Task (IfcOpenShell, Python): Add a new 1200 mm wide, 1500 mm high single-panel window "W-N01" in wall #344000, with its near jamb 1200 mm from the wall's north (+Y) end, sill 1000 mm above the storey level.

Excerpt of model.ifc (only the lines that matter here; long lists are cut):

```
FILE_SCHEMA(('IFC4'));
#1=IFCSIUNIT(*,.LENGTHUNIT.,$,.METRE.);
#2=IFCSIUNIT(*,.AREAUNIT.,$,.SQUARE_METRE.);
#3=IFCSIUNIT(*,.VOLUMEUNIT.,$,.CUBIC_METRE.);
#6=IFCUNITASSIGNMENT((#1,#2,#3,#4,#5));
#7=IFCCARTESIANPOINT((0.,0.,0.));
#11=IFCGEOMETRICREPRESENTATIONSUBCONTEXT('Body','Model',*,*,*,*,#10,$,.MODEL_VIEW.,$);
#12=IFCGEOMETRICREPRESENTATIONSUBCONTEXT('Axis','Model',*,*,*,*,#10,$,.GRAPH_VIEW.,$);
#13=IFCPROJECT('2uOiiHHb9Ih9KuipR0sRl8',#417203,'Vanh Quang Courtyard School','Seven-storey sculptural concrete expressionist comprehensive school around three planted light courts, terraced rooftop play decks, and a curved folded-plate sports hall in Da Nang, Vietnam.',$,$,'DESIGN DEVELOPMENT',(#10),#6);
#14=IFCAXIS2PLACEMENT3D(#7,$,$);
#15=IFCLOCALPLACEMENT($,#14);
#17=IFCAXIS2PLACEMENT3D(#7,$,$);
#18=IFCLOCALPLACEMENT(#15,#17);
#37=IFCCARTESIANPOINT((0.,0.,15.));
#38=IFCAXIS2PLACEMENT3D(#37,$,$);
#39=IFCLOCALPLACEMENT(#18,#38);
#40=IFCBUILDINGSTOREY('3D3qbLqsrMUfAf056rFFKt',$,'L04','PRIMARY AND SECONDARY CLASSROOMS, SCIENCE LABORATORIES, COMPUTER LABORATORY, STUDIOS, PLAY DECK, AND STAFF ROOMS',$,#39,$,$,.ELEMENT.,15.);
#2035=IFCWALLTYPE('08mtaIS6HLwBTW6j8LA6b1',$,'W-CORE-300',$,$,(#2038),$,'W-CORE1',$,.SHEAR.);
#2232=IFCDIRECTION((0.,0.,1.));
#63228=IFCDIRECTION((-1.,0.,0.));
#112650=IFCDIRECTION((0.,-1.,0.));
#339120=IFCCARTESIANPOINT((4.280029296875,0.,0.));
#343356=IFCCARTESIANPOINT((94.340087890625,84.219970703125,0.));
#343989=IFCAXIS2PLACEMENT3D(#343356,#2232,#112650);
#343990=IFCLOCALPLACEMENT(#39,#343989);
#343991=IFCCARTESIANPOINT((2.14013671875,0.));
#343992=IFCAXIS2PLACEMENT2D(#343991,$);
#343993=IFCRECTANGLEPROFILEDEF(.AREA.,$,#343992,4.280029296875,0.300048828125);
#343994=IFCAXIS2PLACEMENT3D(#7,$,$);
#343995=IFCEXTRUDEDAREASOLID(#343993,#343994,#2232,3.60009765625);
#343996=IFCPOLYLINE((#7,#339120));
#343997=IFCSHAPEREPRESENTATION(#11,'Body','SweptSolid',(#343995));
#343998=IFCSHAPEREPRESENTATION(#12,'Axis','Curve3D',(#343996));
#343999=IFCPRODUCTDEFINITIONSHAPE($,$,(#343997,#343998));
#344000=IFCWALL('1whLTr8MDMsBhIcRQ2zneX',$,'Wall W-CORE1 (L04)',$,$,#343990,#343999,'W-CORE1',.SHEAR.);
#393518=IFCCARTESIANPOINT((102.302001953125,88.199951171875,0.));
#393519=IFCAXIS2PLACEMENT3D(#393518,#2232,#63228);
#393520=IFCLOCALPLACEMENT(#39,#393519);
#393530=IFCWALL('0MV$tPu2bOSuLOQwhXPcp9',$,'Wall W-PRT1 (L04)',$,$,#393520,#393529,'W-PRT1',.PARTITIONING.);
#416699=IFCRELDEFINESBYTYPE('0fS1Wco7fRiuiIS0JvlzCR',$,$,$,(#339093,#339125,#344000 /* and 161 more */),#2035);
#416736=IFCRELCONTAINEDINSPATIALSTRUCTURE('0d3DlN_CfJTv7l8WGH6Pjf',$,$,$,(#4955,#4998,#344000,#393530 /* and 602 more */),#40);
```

```python
import numpy as np
import ifcopenshell
import ifcopenshell.api.feature
import ifcopenshell.api.geometry
import ifcopenshell.api.root
import ifcopenshell.api.spatial
import ifcopenshell.geom
import ifcopenshell.util.element
import ifcopenshell.util.placement
import ifcopenshell.util.representation
import ifcopenshell.util.shape
import ifcopenshell.util.unit

model = ifcopenshell.open("model.ifc")
unit_scale = ifcopenshell.util.unit.calculate_unit_scale(model)
settings = ifcopenshell.geom.settings()


def volume(element):
    """Net volume in cubic metres, openings subtracted."""
    shape = ifcopenshell.geom.create_shape(settings, element)
    return ifcopenshell.util.shape.get_volume(shape.geometry)


wall = model.by_guid("1whLTr8MDMsBhIcRQ2zneX")
storey = ifcopenshell.util.element.get_container(wall, ifc_class="IfcBuildingStorey")
context = ifcopenshell.util.representation.get_context(model, "Model", "Body", "MODEL_VIEW")
before = volume(wall)

width, height, from_end, sill = 1.2, 1.5, 1.2, 1  # metres

# The wall runs along its own X axis, and the end named is its -X end.
wall_shape = ifcopenshell.geom.create_shape(settings, wall)
x, y, z = ifcopenshell.util.shape.get_vertices(wall_shape.geometry).T
start = x.min() + from_end
face, thickness = float(y.min()), float(y.max() - y.min())
wall_matrix = ifcopenshell.util.placement.get_local_placement(wall.ObjectPlacement)
level = ifcopenshell.util.placement.get_local_placement(storey.ObjectPlacement)[2, 3]


def in_wall(x, y):
    """Placement at x, y metres in the wall's axes, at sill height."""
    matrix = wall_matrix.copy()
    matrix[:, 3] = wall_matrix @ np.array([x / unit_scale, y / unit_scale, 0.0, 1.0])
    matrix[2, 3] = level + sill / unit_scale
    return matrix


# Opening: a box that overshoots both wall faces by 50 mm.
opening = ifcopenshell.api.root.create_entity(model, ifc_class="IfcOpeningElement", predefined_type="OPENING")
box = ifcopenshell.api.geometry.add_wall_representation(
    model, context=context, length=width, height=height, thickness=thickness + 0.1
)
ifcopenshell.api.geometry.assign_representation(model, product=opening, representation=box)
ifcopenshell.api.geometry.edit_object_placement(model, product=opening, matrix=in_wall(start, face - 0.05), is_si=False)
ifcopenshell.api.feature.add_feature(model, feature=opening, element=wall)

window = ifcopenshell.api.root.create_entity(model, ifc_class="IfcWindow", name="W-N01", predefined_type="WINDOW")
window.OverallWidth, window.OverallHeight = width / unit_scale, height / unit_scale
window.PartitioningType = "SINGLE_PANEL"
body = ifcopenshell.api.geometry.add_window_representation(
    model,
    context=context,
    overall_width=window.OverallWidth,
    overall_height=window.OverallHeight,
    partition_type="SINGLE_PANEL",
)
ifcopenshell.api.geometry.assign_representation(model, product=window, representation=body)
ifcopenshell.api.spatial.assign_container(model, products=[window], relating_structure=storey)
ifcopenshell.api.feature.add_filling(model, opening=opening, element=window)

# Centre the window in the wall's thickness.
ifcopenshell.api.geometry.edit_object_placement(model, product=window, matrix=in_wall(start, face), is_si=False)
window_shape = ifcopenshell.geom.create_shape(settings, window)
depth = ifcopenshell.util.shape.get_vertices(window_shape.geometry)[:, 1]
offset = face + thickness / 2 - (depth.min() + depth.max()) / 2
ifcopenshell.api.geometry.edit_object_placement(model, product=window, matrix=in_wall(start, offset), is_si=False)

after = volume(wall)

print(f"wall volume {before:.3f} -> {after:.3f} m3")

model.write("model_updated.ifc")
```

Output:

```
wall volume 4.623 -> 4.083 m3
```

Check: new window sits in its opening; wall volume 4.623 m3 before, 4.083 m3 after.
